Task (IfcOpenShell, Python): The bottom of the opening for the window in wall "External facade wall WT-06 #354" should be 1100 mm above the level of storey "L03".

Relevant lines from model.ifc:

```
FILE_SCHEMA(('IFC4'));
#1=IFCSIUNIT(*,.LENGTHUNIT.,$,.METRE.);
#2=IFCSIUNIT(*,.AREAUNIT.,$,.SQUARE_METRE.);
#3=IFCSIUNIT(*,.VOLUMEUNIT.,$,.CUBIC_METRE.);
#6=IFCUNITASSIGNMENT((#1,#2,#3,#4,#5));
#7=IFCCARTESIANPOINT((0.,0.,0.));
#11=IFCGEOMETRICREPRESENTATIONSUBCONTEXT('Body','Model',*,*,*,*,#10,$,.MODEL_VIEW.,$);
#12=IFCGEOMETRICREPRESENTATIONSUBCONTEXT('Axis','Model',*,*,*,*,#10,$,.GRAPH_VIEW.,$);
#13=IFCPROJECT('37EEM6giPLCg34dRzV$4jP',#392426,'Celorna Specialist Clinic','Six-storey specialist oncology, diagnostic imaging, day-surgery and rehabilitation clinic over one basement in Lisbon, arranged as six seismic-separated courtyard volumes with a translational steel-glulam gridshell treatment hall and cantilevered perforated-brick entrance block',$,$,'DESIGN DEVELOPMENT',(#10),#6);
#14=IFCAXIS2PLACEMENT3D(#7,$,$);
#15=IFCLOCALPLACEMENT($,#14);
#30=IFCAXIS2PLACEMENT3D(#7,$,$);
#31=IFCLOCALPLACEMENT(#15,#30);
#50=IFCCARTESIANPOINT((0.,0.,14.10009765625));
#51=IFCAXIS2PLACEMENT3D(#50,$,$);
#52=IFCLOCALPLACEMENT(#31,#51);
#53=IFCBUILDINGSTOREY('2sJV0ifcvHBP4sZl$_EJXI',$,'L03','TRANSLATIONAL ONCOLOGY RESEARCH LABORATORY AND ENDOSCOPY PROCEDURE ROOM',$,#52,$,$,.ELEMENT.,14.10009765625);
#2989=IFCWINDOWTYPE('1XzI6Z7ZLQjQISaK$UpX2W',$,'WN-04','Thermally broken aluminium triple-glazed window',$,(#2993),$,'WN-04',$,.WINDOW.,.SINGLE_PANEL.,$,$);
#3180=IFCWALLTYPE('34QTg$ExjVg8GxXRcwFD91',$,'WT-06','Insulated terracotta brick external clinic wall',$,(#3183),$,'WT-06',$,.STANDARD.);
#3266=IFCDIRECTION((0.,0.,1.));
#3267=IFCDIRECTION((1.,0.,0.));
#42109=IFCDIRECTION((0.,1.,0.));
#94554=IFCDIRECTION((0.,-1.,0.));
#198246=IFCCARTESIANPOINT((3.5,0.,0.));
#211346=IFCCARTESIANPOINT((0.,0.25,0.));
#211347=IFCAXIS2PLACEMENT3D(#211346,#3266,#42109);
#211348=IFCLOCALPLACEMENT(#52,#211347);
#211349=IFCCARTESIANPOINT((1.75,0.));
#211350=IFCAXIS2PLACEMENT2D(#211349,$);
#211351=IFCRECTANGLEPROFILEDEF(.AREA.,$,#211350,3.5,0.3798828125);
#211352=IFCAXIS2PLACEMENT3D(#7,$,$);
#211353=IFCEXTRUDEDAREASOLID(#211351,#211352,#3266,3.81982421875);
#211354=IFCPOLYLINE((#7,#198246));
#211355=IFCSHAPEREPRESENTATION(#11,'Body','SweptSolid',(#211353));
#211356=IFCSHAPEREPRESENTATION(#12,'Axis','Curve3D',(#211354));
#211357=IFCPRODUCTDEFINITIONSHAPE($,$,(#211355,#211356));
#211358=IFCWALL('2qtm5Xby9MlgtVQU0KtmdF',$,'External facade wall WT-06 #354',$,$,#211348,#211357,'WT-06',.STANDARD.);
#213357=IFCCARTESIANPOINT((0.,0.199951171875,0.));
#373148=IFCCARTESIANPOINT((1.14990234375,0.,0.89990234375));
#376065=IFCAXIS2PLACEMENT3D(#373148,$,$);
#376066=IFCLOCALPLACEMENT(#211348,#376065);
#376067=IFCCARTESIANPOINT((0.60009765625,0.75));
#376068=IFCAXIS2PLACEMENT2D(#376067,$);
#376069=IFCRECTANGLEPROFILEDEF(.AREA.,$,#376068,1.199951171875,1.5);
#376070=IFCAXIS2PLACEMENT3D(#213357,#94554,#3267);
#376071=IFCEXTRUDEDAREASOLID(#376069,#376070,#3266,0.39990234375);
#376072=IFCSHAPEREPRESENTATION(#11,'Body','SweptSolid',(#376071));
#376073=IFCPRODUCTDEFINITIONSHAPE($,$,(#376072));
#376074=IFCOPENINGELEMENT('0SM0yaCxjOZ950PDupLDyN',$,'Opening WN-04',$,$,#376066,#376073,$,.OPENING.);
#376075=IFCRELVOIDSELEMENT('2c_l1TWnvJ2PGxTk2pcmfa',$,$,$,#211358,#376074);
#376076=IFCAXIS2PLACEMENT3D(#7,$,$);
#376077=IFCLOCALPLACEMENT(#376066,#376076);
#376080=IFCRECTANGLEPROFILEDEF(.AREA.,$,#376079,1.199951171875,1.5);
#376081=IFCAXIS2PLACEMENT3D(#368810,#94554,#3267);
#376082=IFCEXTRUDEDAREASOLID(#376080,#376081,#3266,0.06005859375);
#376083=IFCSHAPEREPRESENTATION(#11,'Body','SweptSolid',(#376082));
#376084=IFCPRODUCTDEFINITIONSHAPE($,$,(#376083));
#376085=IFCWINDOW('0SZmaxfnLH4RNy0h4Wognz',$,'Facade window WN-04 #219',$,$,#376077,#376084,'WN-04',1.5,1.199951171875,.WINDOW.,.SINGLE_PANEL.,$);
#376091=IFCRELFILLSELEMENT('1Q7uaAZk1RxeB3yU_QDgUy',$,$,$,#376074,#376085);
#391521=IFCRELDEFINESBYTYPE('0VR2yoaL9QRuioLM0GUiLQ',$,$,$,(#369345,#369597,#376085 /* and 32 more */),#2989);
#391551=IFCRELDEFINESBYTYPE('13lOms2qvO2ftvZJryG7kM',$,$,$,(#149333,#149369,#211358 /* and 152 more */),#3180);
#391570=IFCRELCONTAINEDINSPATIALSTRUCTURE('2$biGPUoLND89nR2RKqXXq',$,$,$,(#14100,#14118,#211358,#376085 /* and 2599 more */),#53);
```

```python
import numpy as np
import ifcopenshell
import ifcopenshell.api.geometry
import ifcopenshell.geom
import ifcopenshell.util.element
import ifcopenshell.util.placement
import ifcopenshell.util.shape
import ifcopenshell.util.unit

model = ifcopenshell.open("model.ifc")
unit_scale = ifcopenshell.util.unit.calculate_unit_scale(model)

window = model.by_id(376085)
opening = window.FillsVoids[0].RelatingOpeningElement
storey = ifcopenshell.util.element.get_container(window, ifc_class="IfcBuildingStorey")
level = ifcopenshell.util.placement.get_local_placement(storey.ObjectPlacement)[2, 3]

# The opening's origin need not be at the sill, so measure its lowest point.
shape = ifcopenshell.geom.create_shape(ifcopenshell.geom.settings(), opening)
bottom = ifcopenshell.util.shape.get_shape_bottom_elevation(shape, shape.geometry) / unit_scale
dz = level + 1.1 / unit_scale - bottom

shift = np.array([0.0, 0.0, dz])
# The window is placed relative to its opening, so it follows when the opening moves.
matrix = ifcopenshell.util.placement.get_local_placement(opening.ObjectPlacement)
matrix[:3, 3] += shift
ifcopenshell.api.geometry.edit_object_placement(
    model, product=opening, matrix=matrix, is_si=False, should_transform_children=True
)

print(f"moved by {dz * unit_scale:+.3f} m")

model.write("model-out.ifc")
```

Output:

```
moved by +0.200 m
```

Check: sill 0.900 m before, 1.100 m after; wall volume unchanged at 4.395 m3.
